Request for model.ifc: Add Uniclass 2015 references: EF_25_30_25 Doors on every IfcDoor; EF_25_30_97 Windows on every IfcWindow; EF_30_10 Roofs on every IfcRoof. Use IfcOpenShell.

First a look at what the model holds.

```python
import ifcopenshell

model = ifcopenshell.open("model.ifc")
print(model.schema)
print("classifications:", [c.Name for c in model.by_type("IfcClassification")])
for ifc_class in ("IfcDoor", "IfcRoof", "IfcStair", "IfcWall", "IfcWindow"):
    print(ifc_class, len(model.by_type(ifc_class)))
```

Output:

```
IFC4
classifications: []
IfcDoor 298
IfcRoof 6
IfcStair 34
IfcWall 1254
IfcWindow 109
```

```python
import ifcopenshell
import ifcopenshell.api.classification

model = ifcopenshell.open("model.ifc")

system = ifcopenshell.api.classification.add_classification(model, classification="Uniclass 2015")

codes = {
    "IfcDoor": ("EF_25_30_25", "Doors"),
    "IfcWindow": ("EF_25_30_97", "Windows"),
    "IfcRoof": ("EF_30_10", "Roofs"),
}
for ifc_class, (code, name) in codes.items():
    products = model.by_type(ifc_class)
    ifcopenshell.api.classification.add_reference(
        model, products=products, classification=system, identification=code, name=name
    )
    print(code, len(products))

model.write("model_rev.ifc")
```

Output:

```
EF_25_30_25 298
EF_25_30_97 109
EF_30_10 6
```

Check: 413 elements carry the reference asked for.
